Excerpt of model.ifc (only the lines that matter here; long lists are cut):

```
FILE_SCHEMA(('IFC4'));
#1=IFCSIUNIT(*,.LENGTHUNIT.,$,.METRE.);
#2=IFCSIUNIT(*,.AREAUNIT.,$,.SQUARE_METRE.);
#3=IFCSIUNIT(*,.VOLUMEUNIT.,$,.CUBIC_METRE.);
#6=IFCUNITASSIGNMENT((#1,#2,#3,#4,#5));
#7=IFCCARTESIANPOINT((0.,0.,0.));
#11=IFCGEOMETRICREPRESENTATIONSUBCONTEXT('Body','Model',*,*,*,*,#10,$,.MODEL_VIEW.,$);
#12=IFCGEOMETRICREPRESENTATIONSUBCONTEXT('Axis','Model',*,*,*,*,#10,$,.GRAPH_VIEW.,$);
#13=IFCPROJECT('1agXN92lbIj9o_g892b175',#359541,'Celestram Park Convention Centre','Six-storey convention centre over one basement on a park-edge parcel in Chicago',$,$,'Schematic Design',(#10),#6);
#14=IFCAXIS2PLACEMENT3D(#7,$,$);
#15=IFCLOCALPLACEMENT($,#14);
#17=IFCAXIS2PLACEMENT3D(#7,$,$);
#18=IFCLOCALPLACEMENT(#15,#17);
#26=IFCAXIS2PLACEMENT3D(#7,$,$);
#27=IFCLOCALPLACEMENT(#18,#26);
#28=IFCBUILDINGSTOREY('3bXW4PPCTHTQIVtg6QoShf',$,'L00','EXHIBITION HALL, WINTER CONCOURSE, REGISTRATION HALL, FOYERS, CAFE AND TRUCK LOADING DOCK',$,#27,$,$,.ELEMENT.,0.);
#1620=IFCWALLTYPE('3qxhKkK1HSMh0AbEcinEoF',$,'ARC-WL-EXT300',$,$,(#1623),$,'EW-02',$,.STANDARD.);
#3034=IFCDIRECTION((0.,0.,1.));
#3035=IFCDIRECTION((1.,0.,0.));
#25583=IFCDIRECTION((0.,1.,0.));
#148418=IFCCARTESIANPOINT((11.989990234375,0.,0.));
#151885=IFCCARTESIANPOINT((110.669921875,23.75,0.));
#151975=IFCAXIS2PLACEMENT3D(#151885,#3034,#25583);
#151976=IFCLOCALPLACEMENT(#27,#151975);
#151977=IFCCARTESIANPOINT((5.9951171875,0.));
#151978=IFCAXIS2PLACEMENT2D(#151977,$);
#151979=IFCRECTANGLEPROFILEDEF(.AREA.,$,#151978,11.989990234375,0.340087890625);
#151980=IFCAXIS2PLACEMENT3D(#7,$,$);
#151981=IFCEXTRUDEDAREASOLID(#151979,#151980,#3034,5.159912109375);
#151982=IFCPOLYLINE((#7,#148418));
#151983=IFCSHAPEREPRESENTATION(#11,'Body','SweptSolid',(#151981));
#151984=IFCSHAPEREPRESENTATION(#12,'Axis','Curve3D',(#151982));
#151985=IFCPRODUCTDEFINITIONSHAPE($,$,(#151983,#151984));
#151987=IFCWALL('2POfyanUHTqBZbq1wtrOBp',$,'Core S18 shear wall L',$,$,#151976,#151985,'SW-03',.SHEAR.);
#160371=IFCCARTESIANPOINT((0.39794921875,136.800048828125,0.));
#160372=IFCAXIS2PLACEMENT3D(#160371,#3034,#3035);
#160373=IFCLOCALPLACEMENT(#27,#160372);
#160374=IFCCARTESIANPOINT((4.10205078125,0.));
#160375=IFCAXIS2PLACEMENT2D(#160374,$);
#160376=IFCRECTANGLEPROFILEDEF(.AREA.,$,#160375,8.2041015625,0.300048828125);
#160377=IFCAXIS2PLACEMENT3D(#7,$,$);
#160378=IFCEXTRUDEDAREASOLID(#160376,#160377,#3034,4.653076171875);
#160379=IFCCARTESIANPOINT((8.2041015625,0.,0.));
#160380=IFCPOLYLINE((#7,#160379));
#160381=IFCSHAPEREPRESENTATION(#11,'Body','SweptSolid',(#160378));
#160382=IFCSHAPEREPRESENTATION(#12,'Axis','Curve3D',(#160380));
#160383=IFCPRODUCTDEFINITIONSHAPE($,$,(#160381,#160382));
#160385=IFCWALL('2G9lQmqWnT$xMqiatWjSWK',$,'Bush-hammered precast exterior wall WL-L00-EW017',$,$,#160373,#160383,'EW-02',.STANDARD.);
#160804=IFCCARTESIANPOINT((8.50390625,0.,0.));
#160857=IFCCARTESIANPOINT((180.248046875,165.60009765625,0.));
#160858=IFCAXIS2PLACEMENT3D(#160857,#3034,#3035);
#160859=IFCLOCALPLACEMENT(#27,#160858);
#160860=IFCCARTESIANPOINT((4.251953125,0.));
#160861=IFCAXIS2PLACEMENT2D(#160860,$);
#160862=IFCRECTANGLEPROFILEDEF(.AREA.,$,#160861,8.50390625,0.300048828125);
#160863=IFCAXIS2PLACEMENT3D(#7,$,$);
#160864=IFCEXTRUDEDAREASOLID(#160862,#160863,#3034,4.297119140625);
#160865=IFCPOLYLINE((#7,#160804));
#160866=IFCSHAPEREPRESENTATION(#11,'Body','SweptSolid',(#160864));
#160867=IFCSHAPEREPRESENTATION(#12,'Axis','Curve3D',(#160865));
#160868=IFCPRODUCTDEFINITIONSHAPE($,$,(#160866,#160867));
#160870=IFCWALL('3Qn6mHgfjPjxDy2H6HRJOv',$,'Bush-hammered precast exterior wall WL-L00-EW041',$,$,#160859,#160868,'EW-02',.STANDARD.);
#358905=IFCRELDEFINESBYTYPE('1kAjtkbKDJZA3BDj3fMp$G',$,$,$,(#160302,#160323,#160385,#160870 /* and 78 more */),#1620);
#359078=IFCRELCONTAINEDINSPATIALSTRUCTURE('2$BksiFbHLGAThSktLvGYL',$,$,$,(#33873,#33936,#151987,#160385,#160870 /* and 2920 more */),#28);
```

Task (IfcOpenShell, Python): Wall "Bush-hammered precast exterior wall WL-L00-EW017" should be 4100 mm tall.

```python
import ifcopenshell
import ifcopenshell.geom
import ifcopenshell.util.representation
import ifcopenshell.util.shape

model = ifcopenshell.open("model.ifc")
settings = ifcopenshell.geom.settings()


def volume(element):
    """Net volume in cubic metres, openings subtracted."""
    shape = ifcopenshell.geom.create_shape(settings, element)
    return ifcopenshell.util.shape.get_volume(shape.geometry)


wall = model.by_guid("2G9lQmqWnT$xMqiatWjSWK")
before = volume(wall)

body = ifcopenshell.util.representation.get_representation(wall, "Model", "Body")
solid = body.Items[0]
old_height = solid.Depth
solid.Depth = 4.1
after = volume(wall)

print(f"height {old_height:g} -> {solid.Depth:g}, volume {before:.3f} -> {after:.3f} m3")

model.write("model_updated.ifc")
```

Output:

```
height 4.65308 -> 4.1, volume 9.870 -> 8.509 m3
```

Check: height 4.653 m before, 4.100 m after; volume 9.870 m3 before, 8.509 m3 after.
